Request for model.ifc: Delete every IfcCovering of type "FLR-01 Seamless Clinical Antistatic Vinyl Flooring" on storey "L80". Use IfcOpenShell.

First a look at what the model holds.

```python
import ifcopenshell
import ifcopenshell.util.element

model = ifcopenshell.open("model.ifc")
print(model.schema)
storey = next(s for s in model.by_type("IfcBuildingStorey") if s.Name == "L80")
coverings = [e for e in ifcopenshell.util.element.get_decomposition(storey) if e.is_a("IfcCovering")]
seen = {}
for e in coverings:
    element_type = ifcopenshell.util.element.get_type(e)
    name = element_type.Name if element_type not in (None, e) else None
    seen[name] = seen.get(name, 0) + 1
for name, count in sorted(seen.items(), key=str):
    print(count, "x", name)
```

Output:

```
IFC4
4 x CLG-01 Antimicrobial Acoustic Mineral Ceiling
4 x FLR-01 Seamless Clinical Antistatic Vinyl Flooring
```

```python
import ifcopenshell
import ifcopenshell.api.root
import ifcopenshell.util.element

model = ifcopenshell.open("model.ifc")

storey = next(s for s in model.by_type("IfcBuildingStorey") if s.Name == "L80")
coverings = [e for e in ifcopenshell.util.element.get_decomposition(storey) if e.is_a("IfcCovering")]
targets = [e for e in coverings if (t := ifcopenshell.util.element.get_type(e)) not in (None, e) and t.Name == "FLR-01 Seamless Clinical Antistatic Vinyl Flooring"]

for e in targets:
    ifcopenshell.api.root.remove_product(model, product=e)
print(len(targets), "removed")

model.write("model_updated.ifc")
```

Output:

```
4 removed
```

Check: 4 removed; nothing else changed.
